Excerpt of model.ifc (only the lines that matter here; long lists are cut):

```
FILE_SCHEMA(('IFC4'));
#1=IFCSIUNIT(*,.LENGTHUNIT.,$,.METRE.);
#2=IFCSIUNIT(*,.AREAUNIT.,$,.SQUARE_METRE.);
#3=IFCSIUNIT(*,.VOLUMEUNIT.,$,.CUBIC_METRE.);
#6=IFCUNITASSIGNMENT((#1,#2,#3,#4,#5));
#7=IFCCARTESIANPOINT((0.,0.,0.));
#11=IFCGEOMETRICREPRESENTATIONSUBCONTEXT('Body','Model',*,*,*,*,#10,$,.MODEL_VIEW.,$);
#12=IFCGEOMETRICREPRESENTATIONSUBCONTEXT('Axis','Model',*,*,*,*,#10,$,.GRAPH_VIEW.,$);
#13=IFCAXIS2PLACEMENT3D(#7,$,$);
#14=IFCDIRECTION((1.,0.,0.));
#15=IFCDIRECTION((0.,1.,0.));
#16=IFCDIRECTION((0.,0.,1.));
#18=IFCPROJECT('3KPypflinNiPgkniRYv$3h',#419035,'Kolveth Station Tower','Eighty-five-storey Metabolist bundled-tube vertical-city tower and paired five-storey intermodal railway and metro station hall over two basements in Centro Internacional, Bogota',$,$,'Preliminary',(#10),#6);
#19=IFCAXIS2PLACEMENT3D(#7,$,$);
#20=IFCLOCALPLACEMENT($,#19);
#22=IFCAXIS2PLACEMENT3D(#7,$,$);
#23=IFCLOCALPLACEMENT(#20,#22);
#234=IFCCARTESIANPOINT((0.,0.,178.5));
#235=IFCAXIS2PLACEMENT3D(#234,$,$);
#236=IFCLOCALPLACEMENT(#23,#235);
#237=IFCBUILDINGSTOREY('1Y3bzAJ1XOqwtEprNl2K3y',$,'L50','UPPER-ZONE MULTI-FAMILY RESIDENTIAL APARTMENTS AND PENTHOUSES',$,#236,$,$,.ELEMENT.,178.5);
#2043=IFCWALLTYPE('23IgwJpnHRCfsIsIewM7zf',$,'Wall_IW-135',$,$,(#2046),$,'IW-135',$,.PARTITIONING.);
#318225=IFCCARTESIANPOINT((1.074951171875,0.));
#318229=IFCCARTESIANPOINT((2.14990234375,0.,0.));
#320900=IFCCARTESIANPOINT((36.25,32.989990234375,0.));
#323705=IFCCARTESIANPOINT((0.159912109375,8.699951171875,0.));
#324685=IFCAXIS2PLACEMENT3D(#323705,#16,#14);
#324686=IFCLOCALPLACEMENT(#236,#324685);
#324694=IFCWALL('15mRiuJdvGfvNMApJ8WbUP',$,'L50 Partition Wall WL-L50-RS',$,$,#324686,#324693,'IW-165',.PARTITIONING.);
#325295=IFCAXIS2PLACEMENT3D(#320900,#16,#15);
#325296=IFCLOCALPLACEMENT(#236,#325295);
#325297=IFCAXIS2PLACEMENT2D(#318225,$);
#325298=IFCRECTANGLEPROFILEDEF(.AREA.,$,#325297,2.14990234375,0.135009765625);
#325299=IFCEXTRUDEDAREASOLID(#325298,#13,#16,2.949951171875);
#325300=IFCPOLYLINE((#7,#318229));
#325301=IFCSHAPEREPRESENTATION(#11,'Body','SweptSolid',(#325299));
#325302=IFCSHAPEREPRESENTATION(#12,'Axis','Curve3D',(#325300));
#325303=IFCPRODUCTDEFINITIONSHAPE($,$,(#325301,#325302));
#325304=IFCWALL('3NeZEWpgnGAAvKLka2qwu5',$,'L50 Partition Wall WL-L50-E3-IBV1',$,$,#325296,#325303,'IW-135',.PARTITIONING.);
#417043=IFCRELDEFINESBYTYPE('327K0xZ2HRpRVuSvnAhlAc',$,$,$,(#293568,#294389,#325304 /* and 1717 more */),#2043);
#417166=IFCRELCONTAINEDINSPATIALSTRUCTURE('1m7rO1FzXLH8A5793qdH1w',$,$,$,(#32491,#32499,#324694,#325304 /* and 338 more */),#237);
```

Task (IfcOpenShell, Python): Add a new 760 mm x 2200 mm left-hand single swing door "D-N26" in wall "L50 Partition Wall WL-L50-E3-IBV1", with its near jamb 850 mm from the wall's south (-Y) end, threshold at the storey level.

```python
import numpy as np
import ifcopenshell
import ifcopenshell.api.feature
import ifcopenshell.api.geometry
import ifcopenshell.api.root
import ifcopenshell.api.spatial
import ifcopenshell.geom
import ifcopenshell.util.element
import ifcopenshell.util.placement
import ifcopenshell.util.representation
import ifcopenshell.util.shape
import ifcopenshell.util.unit

model = ifcopenshell.open("model.ifc")
unit_scale = ifcopenshell.util.unit.calculate_unit_scale(model)
settings = ifcopenshell.geom.settings()


def volume(element):
    """Net volume in cubic metres, openings subtracted."""
    shape = ifcopenshell.geom.create_shape(settings, element)
    return ifcopenshell.util.shape.get_volume(shape.geometry)


wall = model.by_guid("3NeZEWpgnGAAvKLka2qwu5")
storey = ifcopenshell.util.element.get_container(wall, ifc_class="IfcBuildingStorey")
context = ifcopenshell.util.representation.get_context(model, "Model", "Body", "MODEL_VIEW")
before = volume(wall)

width, height, from_end, sill = 0.76, 2.2, 0.85, 0.0  # metres

# The wall runs along its own X axis, and the end named is its -X end.
wall_shape = ifcopenshell.geom.create_shape(settings, wall)
x, y, z = ifcopenshell.util.shape.get_vertices(wall_shape.geometry).T
start = x.min() + from_end
face, thickness = float(y.min()), float(y.max() - y.min())
wall_matrix = ifcopenshell.util.placement.get_local_placement(wall.ObjectPlacement)
level = ifcopenshell.util.placement.get_local_placement(storey.ObjectPlacement)[2, 3]


def in_wall(x, y):
    """Placement at x, y metres in the wall's axes, at sill height."""
    matrix = wall_matrix.copy()
    matrix[:, 3] = wall_matrix @ np.array([x / unit_scale, y / unit_scale, 0.0, 1.0])
    matrix[2, 3] = level + sill / unit_scale
    return matrix


# Opening: a box that overshoots both wall faces by 50 mm.
opening = ifcopenshell.api.root.create_entity(model, ifc_class="IfcOpeningElement", predefined_type="OPENING")
box = ifcopenshell.api.geometry.add_wall_representation(
    model, context=context, length=width, height=height, thickness=thickness + 0.1
)
ifcopenshell.api.geometry.assign_representation(model, product=opening, representation=box)
ifcopenshell.api.geometry.edit_object_placement(model, product=opening, matrix=in_wall(start, face - 0.05), is_si=False)
ifcopenshell.api.feature.add_feature(model, feature=opening, element=wall)

door = ifcopenshell.api.root.create_entity(model, ifc_class="IfcDoor", name="D-N26", predefined_type="DOOR")
door.OverallWidth, door.OverallHeight = width / unit_scale, height / unit_scale
door.OperationType = "SINGLE_SWING_LEFT"
body = ifcopenshell.api.geometry.add_door_representation(
    model,
    context=context,
    overall_width=door.OverallWidth,
    overall_height=door.OverallHeight,
    operation_type="SINGLE_SWING_LEFT",
    lining_properties={"LiningDepth": thickness / unit_scale, "ThresholdDepth": thickness / unit_scale},
)
ifcopenshell.api.geometry.assign_representation(model, product=door, representation=body)
ifcopenshell.api.spatial.assign_container(model, products=[door], relating_structure=storey)
ifcopenshell.api.feature.add_filling(model, opening=opening, element=door)

# The lining spans the wall, so the door starts at the wall face.
ifcopenshell.api.geometry.edit_object_placement(model, product=door, matrix=in_wall(start, face), is_si=False)

after = volume(wall)

print(f"wall volume {before:.3f} -> {after:.3f} m3")

model.write("model_v2.ifc")
```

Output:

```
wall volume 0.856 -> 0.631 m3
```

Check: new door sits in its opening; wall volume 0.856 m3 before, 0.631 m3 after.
